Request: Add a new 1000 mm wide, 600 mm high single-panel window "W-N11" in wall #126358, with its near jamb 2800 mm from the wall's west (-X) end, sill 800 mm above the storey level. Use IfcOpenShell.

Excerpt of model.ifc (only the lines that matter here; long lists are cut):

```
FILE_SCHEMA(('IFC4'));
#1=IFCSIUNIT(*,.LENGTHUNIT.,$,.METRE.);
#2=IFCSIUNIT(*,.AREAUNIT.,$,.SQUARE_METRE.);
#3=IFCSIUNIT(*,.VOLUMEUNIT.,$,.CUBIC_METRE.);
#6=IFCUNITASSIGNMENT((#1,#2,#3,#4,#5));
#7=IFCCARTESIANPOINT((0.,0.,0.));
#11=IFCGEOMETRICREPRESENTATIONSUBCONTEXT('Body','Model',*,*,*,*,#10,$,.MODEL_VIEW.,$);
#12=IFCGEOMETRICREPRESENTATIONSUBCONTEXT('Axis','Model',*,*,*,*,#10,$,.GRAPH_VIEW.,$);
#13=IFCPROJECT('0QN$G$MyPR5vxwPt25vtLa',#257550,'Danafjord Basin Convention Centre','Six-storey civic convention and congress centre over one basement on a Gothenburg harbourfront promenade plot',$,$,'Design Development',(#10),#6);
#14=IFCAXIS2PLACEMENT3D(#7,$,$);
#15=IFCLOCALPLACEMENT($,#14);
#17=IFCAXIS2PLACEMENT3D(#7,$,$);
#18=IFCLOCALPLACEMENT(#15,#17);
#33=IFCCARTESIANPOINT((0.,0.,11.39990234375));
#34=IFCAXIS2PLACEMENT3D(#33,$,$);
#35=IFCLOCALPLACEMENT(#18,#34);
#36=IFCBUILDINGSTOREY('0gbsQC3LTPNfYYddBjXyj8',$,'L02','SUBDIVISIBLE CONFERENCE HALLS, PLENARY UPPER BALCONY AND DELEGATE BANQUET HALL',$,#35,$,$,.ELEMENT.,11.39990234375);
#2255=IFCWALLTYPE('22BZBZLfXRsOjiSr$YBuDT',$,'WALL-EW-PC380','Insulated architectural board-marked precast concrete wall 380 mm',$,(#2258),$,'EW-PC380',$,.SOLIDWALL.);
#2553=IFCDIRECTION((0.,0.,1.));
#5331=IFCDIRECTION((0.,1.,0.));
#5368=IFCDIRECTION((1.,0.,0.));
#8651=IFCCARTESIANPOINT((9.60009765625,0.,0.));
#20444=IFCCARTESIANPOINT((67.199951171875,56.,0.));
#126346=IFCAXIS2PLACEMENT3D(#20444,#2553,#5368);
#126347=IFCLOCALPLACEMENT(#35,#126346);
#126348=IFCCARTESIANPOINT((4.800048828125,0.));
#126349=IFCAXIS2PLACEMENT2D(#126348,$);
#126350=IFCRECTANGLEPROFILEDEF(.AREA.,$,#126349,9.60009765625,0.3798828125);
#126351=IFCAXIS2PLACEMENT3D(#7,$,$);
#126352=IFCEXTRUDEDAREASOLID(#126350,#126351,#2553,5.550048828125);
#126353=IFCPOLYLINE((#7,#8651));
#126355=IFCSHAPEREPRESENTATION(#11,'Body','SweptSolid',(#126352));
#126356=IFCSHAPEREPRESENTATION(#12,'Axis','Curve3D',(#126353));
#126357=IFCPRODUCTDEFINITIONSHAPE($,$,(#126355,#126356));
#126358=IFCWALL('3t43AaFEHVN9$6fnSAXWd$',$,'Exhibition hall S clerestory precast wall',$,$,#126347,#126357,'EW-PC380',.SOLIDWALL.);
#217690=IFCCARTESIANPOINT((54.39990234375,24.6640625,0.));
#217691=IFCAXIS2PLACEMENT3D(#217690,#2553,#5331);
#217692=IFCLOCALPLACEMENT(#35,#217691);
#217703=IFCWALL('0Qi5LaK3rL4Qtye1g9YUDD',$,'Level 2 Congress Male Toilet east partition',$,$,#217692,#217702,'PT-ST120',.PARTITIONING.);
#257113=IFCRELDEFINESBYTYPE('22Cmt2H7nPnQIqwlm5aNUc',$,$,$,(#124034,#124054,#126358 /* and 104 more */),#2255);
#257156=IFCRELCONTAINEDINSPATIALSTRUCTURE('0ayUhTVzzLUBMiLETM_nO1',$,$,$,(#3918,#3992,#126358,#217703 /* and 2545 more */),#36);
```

```python
import numpy as np
import ifcopenshell
import ifcopenshell.api.feature
import ifcopenshell.api.geometry
import ifcopenshell.api.root
import ifcopenshell.api.spatial
import ifcopenshell.geom
import ifcopenshell.util.element
import ifcopenshell.util.placement
import ifcopenshell.util.representation
import ifcopenshell.util.shape
import ifcopenshell.util.unit

model = ifcopenshell.open("model.ifc")
unit_scale = ifcopenshell.util.unit.calculate_unit_scale(model)
settings = ifcopenshell.geom.settings()


def volume(element):
    """Net volume in cubic metres, openings subtracted."""
    shape = ifcopenshell.geom.create_shape(settings, element)
    return ifcopenshell.util.shape.get_volume(shape.geometry)


wall = model.by_guid("3t43AaFEHVN9$6fnSAXWd$")
storey = ifcopenshell.util.element.get_container(wall, ifc_class="IfcBuildingStorey")
context = ifcopenshell.util.representation.get_context(model, "Model", "Body", "MODEL_VIEW")
before = volume(wall)

width, height, from_end, sill = 1, 0.6, 2.8, 0.8  # metres

# The wall runs along its own X axis, and the end named is its -X end.
wall_shape = ifcopenshell.geom.create_shape(settings, wall)
x, y, z = ifcopenshell.util.shape.get_vertices(wall_shape.geometry).T
start = x.min() + from_end
face, thickness = float(y.min()), float(y.max() - y.min())
wall_matrix = ifcopenshell.util.placement.get_local_placement(wall.ObjectPlacement)
level = ifcopenshell.util.placement.get_local_placement(storey.ObjectPlacement)[2, 3]


def in_wall(x, y):
    """Placement at x, y metres in the wall's axes, at sill height."""
    matrix = wall_matrix.copy()
    matrix[:, 3] = wall_matrix @ np.array([x / unit_scale, y / unit_scale, 0.0, 1.0])
    matrix[2, 3] = level + sill / unit_scale
    return matrix


# Opening: a box that overshoots both wall faces by 50 mm.
opening = ifcopenshell.api.root.create_entity(model, ifc_class="IfcOpeningElement", predefined_type="OPENING")
box = ifcopenshell.api.geometry.add_wall_representation(
    model, context=context, length=width, height=height, thickness=thickness + 0.1
)
ifcopenshell.api.geometry.assign_representation(model, product=opening, representation=box)
ifcopenshell.api.geometry.edit_object_placement(model, product=opening, matrix=in_wall(start, face - 0.05), is_si=False)
ifcopenshell.api.feature.add_feature(model, feature=opening, element=wall)

window = ifcopenshell.api.root.create_entity(model, ifc_class="IfcWindow", name="W-N11", predefined_type="WINDOW")
window.OverallWidth, window.OverallHeight = width / unit_scale, height / unit_scale
window.PartitioningType = "SINGLE_PANEL"
body = ifcopenshell.api.geometry.add_window_representation(
    model,
    context=context,
    overall_width=window.OverallWidth,
    overall_height=window.OverallHeight,
    partition_type="SINGLE_PANEL",
)
ifcopenshell.api.geometry.assign_representation(model, product=window, representation=body)
ifcopenshell.api.spatial.assign_container(model, products=[window], relating_structure=storey)
ifcopenshell.api.feature.add_filling(model, opening=opening, element=window)

# Centre the window in the wall's thickness.
ifcopenshell.api.geometry.edit_object_placement(model, product=window, matrix=in_wall(start, face), is_si=False)
window_shape = ifcopenshell.geom.create_shape(settings, window)
depth = ifcopenshell.util.shape.get_vertices(window_shape.geometry)[:, 1]
offset = face + thickness / 2 - (depth.min() + depth.max()) / 2
ifcopenshell.api.geometry.edit_object_placement(model, product=window, matrix=in_wall(start, offset), is_si=False)

after = volume(wall)

print(f"wall volume {before:.3f} -> {after:.3f} m3")

model.write("model_updated.ifc")
```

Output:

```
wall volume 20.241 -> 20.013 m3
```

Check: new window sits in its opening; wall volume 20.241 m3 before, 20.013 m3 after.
